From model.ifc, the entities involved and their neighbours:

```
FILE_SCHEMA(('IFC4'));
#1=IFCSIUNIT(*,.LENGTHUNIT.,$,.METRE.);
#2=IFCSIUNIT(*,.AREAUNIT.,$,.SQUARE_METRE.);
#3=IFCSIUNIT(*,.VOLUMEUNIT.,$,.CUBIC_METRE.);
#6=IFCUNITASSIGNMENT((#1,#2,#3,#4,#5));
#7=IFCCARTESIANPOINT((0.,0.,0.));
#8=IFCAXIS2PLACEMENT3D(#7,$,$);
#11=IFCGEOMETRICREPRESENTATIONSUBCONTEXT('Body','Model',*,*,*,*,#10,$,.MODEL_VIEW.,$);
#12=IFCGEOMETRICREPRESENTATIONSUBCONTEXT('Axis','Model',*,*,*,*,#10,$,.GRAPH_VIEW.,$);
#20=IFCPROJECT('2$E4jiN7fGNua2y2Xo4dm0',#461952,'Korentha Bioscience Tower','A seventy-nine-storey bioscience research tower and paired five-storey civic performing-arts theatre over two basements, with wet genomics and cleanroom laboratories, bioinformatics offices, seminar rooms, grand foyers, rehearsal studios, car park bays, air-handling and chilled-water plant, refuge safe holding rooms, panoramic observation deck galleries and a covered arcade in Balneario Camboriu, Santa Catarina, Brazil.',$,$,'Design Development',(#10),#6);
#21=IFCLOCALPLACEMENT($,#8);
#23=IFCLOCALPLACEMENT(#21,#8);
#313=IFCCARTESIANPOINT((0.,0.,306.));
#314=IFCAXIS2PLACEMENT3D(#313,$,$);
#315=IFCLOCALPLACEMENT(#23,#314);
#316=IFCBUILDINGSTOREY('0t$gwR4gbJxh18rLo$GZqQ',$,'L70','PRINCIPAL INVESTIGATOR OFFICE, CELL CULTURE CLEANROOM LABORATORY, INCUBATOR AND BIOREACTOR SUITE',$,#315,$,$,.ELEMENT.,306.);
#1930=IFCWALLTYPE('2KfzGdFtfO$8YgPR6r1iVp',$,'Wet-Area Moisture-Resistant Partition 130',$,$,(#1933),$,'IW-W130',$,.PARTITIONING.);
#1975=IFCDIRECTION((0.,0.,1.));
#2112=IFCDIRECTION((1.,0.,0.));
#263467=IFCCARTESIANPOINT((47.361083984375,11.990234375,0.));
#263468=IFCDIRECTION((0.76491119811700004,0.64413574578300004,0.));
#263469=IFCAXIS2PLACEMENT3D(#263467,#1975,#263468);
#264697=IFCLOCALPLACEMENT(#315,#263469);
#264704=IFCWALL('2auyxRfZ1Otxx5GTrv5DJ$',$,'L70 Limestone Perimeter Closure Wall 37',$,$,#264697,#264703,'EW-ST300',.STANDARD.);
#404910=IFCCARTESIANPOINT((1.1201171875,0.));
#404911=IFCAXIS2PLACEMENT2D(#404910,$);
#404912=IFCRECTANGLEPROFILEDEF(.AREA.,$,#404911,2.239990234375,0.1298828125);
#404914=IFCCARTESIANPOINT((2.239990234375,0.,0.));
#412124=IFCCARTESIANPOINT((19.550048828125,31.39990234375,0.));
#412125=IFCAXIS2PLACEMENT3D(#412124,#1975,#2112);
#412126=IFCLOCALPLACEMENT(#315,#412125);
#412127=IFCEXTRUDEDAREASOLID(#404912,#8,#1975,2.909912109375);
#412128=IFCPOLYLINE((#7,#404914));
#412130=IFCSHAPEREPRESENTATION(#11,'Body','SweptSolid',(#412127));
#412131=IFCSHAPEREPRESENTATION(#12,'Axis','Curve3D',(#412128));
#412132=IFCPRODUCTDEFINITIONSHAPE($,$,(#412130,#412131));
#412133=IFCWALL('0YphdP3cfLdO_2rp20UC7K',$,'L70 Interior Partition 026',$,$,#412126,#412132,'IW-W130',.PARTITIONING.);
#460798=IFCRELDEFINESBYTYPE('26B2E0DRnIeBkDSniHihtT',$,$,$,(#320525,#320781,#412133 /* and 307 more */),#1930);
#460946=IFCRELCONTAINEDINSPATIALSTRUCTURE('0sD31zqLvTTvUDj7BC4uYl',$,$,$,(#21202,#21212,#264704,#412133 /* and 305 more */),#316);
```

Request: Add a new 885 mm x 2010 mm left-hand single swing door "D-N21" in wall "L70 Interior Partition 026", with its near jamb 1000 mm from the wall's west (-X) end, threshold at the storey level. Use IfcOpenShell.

```python
import numpy as np
import ifcopenshell
import ifcopenshell.api.feature
import ifcopenshell.api.geometry
import ifcopenshell.api.root
import ifcopenshell.api.spatial
import ifcopenshell.geom
import ifcopenshell.util.element
import ifcopenshell.util.placement
import ifcopenshell.util.representation
import ifcopenshell.util.shape
import ifcopenshell.util.unit

model = ifcopenshell.open("model.ifc")
unit_scale = ifcopenshell.util.unit.calculate_unit_scale(model)
settings = ifcopenshell.geom.settings()


def volume(element):
    """Net volume in cubic metres, openings subtracted."""
    shape = ifcopenshell.geom.create_shape(settings, element)
    return ifcopenshell.util.shape.get_volume(shape.geometry)


wall = model.by_id(412133)
storey = ifcopenshell.util.element.get_container(wall, ifc_class="IfcBuildingStorey")
context = ifcopenshell.util.representation.get_context(model, "Model", "Body", "MODEL_VIEW")
before = volume(wall)

width, height, from_end, sill = 0.885, 2.01, 1, 0.0  # metres

# The wall runs along its own X axis, and the end named is its -X end.
wall_shape = ifcopenshell.geom.create_shape(settings, wall)
x, y, z = ifcopenshell.util.shape.get_vertices(wall_shape.geometry).T
start = x.min() + from_end
face, thickness = float(y.min()), float(y.max() - y.min())
wall_matrix = ifcopenshell.util.placement.get_local_placement(wall.ObjectPlacement)
level = ifcopenshell.util.placement.get_local_placement(storey.ObjectPlacement)[2, 3]


def in_wall(x, y):
    """Placement at x, y metres in the wall's axes, at sill height."""
    matrix = wall_matrix.copy()
    matrix[:, 3] = wall_matrix @ np.array([x / unit_scale, y / unit_scale, 0.0, 1.0])
    matrix[2, 3] = level + sill / unit_scale
    return matrix


# Opening: a box that overshoots both wall faces by 50 mm.
opening = ifcopenshell.api.root.create_entity(model, ifc_class="IfcOpeningElement", predefined_type="OPENING")
box = ifcopenshell.api.geometry.add_wall_representation(
    model, context=context, length=width, height=height, thickness=thickness + 0.1
)
ifcopenshell.api.geometry.assign_representation(model, product=opening, representation=box)
ifcopenshell.api.geometry.edit_object_placement(model, product=opening, matrix=in_wall(start, face - 0.05), is_si=False)
ifcopenshell.api.feature.add_feature(model, feature=opening, element=wall)

door = ifcopenshell.api.root.create_entity(model, ifc_class="IfcDoor", name="D-N21", predefined_type="DOOR")
door.OverallWidth, door.OverallHeight = width / unit_scale, height / unit_scale
door.OperationType = "SINGLE_SWING_LEFT"
body = ifcopenshell.api.geometry.add_door_representation(
    model,
    context=context,
    overall_width=door.OverallWidth,
    overall_height=door.OverallHeight,
    operation_type="SINGLE_SWING_LEFT",
    lining_properties={"LiningDepth": thickness / unit_scale, "ThresholdDepth": thickness / unit_scale},
)
ifcopenshell.api.geometry.assign_representation(model, product=door, representation=body)
ifcopenshell.api.spatial.assign_container(model, products=[door], relating_structure=storey)
ifcopenshell.api.feature.add_filling(model, opening=opening, element=door)

# The lining spans the wall, so the door starts at the wall face.
ifcopenshell.api.geometry.edit_object_placement(model, product=door, matrix=in_wall(start, face), is_si=False)

after = volume(wall)

print(f"wall volume {before:.3f} -> {after:.3f} m3")

model.write("model_edited.ifc")
```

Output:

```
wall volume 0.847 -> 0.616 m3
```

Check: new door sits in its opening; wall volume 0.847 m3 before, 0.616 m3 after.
